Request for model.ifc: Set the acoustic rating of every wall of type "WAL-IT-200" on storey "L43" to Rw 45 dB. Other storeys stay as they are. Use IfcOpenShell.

First a look at what the model holds.

```python
import ifcopenshell
import ifcopenshell.util.element

model = ifcopenshell.open("model.ifc")
print(model.schema)
storey = next(s for s in model.by_type("IfcBuildingStorey") if s.Name == "L43")
walls = [e for e in ifcopenshell.util.element.get_decomposition(storey) if e.is_a("IfcWall")]
seen = {}
for e in walls:
    element_type = ifcopenshell.util.element.get_type(e)
    key = (element_type.Name if element_type != e and element_type else None, ifcopenshell.util.element.get_pset(e, "Pset_WallCommon", "AcousticRating"))
    seen[key] = seen.get(key, 0) + 1
for (name, value), count in sorted(seen.items(), key=str):
    print(count, "x", name, "|", value)
```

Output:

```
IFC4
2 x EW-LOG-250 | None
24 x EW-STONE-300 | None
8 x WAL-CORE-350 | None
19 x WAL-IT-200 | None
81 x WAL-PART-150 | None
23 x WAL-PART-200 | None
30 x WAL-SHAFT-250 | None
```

```python
import ifcopenshell
import ifcopenshell.api.pset
import ifcopenshell.util.element

model = ifcopenshell.open("model.ifc")

storey = next(s for s in model.by_type("IfcBuildingStorey") if s.Name == "L43")
walls = [e for e in ifcopenshell.util.element.get_decomposition(storey) if e.is_a("IfcWall")]

count = 0
for e in walls:
    element_type = ifcopenshell.util.element.get_type(e)
    if element_type in (None, e) or element_type.Name != "WAL-IT-200":
        continue
    found = ifcopenshell.util.element.get_pset(e, "Pset_WallCommon", should_inherit=False)
    if found:
        pset = model.by_id(found["id"])
        if len(ifcopenshell.util.element.get_elements_by_pset(pset)) > 1:
            pset = ifcopenshell.api.pset.unshare_pset(model, products=[e], pset=pset)[0]
    else:
        pset = ifcopenshell.api.pset.add_pset(model, product=e, name="Pset_WallCommon")
    ifcopenshell.api.pset.edit_pset(model, pset=pset, properties={"AcousticRating": "Rw 45 dB"})
    count += 1

print(count, "walls updated")

model.write("model_v2.ifc")
```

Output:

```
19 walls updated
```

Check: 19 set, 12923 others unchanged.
